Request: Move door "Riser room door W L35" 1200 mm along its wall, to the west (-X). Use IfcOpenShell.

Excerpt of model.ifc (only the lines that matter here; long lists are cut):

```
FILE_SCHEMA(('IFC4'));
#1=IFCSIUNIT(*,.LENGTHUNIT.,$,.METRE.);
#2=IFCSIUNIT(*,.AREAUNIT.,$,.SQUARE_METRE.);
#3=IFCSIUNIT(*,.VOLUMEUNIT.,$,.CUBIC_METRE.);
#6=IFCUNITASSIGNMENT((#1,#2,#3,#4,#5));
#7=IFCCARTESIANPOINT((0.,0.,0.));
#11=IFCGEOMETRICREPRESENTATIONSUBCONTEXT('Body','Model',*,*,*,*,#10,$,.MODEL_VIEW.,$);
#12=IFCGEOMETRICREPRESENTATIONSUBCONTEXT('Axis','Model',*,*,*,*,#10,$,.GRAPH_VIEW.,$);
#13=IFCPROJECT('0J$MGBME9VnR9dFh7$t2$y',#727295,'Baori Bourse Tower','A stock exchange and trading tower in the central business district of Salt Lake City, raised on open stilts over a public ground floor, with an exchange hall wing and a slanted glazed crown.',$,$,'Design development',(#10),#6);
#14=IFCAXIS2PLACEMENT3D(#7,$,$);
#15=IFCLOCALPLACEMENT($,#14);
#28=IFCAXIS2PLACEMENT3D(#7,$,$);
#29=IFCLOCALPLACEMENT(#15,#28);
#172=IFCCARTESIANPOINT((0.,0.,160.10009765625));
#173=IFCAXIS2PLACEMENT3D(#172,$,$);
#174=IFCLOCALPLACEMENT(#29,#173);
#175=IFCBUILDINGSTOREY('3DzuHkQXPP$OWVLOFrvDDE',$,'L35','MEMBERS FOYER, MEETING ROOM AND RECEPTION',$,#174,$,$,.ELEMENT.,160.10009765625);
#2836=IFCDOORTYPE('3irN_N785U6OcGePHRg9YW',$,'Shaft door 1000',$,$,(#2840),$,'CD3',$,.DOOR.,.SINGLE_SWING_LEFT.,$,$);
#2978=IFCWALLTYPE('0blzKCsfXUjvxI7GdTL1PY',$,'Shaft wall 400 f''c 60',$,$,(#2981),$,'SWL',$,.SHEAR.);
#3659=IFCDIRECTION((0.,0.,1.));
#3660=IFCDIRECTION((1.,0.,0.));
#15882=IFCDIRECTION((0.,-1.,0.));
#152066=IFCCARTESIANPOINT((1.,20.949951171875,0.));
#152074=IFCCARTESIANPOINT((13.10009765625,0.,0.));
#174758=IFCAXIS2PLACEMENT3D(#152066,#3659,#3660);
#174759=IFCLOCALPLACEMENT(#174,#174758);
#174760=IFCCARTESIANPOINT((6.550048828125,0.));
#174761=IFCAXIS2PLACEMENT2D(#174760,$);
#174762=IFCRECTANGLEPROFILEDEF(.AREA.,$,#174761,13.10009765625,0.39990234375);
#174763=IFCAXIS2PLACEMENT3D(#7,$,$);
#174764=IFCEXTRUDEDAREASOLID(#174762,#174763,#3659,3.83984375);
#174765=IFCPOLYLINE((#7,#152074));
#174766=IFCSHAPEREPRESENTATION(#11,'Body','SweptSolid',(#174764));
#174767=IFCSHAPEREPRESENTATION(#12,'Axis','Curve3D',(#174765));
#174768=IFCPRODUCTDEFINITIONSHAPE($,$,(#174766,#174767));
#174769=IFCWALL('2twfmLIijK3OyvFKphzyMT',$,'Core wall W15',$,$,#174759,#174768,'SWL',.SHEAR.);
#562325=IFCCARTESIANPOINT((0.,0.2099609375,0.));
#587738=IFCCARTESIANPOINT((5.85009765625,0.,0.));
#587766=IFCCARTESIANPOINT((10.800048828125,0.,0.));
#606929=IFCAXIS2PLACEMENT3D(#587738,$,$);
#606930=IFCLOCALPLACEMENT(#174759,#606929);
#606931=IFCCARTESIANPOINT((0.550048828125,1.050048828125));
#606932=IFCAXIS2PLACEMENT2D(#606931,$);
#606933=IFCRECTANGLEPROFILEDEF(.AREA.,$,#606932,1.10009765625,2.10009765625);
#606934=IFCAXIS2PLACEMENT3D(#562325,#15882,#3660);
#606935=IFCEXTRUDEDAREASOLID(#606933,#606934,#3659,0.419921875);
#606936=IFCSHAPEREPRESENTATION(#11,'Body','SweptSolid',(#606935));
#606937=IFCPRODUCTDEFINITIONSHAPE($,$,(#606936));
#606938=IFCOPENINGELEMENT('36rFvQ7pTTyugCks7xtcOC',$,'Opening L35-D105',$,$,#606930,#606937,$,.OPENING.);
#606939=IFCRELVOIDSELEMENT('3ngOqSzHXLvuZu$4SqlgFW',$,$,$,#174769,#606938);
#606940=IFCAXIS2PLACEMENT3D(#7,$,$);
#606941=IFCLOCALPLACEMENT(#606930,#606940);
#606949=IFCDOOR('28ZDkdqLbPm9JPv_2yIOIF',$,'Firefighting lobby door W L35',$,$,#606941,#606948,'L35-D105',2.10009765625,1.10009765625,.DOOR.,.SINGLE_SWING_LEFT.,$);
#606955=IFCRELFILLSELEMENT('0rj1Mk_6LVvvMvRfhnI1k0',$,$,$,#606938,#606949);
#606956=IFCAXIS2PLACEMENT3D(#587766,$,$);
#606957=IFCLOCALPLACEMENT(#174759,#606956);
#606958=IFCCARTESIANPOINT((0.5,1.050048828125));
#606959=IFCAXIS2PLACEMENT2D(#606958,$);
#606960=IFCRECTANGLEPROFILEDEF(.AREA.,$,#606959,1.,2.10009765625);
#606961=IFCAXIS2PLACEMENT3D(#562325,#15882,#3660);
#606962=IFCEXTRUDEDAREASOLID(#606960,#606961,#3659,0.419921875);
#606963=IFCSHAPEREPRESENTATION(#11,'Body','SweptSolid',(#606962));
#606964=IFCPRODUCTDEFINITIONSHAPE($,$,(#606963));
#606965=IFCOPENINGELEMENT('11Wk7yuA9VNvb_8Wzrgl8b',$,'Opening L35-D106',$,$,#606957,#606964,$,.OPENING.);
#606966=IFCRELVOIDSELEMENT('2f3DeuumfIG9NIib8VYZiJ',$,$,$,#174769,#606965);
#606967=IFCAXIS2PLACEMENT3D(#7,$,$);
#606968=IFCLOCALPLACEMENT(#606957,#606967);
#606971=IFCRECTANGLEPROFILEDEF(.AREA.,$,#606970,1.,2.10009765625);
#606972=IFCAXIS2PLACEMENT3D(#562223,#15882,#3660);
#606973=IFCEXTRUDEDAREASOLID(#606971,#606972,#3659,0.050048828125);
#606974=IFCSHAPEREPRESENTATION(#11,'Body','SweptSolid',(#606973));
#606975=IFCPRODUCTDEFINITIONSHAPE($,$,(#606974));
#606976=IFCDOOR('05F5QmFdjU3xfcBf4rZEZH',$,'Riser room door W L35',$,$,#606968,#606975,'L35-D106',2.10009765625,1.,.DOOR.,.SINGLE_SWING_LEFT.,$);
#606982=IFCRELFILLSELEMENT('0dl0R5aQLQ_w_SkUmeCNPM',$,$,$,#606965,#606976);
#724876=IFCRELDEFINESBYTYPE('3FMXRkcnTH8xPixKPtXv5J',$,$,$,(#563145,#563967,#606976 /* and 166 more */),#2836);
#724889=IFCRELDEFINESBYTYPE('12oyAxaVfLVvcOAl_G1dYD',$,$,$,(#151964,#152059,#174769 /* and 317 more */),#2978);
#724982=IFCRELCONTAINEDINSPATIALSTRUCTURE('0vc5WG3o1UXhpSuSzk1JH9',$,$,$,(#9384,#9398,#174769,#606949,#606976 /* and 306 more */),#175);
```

```python
import ifcopenshell
import ifcopenshell.api.geometry
import ifcopenshell.util.placement
import ifcopenshell.util.unit

model = ifcopenshell.open("model.ifc")
unit_scale = ifcopenshell.util.unit.calculate_unit_scale(model)

door = model.by_guid("05F5QmFdjU3xfcBf4rZEZH")
opening = door.FillsVoids[0].RelatingOpeningElement
wall = opening.VoidsElements[0].RelatingBuildingElement

wall_matrix = ifcopenshell.util.placement.get_local_placement(wall.ObjectPlacement)
shift = wall_matrix[:3, 0] * -1.2 / unit_scale
before = ifcopenshell.util.placement.get_local_placement(door.ObjectPlacement)[:3, 3].copy()

# The door is placed relative to its opening, so it follows when the opening moves.
matrix = ifcopenshell.util.placement.get_local_placement(opening.ObjectPlacement)
matrix[:3, 3] += shift
ifcopenshell.api.geometry.edit_object_placement(
    model, product=opening, matrix=matrix, is_si=False, should_transform_children=True
)

after = ifcopenshell.util.placement.get_local_placement(door.ObjectPlacement)[:3, 3]
print("door moved by", (after - before).round(3) + 0.0)

model.write("model_v2.ifc")
```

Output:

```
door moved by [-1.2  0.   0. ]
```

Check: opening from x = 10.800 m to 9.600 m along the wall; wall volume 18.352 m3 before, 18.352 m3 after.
